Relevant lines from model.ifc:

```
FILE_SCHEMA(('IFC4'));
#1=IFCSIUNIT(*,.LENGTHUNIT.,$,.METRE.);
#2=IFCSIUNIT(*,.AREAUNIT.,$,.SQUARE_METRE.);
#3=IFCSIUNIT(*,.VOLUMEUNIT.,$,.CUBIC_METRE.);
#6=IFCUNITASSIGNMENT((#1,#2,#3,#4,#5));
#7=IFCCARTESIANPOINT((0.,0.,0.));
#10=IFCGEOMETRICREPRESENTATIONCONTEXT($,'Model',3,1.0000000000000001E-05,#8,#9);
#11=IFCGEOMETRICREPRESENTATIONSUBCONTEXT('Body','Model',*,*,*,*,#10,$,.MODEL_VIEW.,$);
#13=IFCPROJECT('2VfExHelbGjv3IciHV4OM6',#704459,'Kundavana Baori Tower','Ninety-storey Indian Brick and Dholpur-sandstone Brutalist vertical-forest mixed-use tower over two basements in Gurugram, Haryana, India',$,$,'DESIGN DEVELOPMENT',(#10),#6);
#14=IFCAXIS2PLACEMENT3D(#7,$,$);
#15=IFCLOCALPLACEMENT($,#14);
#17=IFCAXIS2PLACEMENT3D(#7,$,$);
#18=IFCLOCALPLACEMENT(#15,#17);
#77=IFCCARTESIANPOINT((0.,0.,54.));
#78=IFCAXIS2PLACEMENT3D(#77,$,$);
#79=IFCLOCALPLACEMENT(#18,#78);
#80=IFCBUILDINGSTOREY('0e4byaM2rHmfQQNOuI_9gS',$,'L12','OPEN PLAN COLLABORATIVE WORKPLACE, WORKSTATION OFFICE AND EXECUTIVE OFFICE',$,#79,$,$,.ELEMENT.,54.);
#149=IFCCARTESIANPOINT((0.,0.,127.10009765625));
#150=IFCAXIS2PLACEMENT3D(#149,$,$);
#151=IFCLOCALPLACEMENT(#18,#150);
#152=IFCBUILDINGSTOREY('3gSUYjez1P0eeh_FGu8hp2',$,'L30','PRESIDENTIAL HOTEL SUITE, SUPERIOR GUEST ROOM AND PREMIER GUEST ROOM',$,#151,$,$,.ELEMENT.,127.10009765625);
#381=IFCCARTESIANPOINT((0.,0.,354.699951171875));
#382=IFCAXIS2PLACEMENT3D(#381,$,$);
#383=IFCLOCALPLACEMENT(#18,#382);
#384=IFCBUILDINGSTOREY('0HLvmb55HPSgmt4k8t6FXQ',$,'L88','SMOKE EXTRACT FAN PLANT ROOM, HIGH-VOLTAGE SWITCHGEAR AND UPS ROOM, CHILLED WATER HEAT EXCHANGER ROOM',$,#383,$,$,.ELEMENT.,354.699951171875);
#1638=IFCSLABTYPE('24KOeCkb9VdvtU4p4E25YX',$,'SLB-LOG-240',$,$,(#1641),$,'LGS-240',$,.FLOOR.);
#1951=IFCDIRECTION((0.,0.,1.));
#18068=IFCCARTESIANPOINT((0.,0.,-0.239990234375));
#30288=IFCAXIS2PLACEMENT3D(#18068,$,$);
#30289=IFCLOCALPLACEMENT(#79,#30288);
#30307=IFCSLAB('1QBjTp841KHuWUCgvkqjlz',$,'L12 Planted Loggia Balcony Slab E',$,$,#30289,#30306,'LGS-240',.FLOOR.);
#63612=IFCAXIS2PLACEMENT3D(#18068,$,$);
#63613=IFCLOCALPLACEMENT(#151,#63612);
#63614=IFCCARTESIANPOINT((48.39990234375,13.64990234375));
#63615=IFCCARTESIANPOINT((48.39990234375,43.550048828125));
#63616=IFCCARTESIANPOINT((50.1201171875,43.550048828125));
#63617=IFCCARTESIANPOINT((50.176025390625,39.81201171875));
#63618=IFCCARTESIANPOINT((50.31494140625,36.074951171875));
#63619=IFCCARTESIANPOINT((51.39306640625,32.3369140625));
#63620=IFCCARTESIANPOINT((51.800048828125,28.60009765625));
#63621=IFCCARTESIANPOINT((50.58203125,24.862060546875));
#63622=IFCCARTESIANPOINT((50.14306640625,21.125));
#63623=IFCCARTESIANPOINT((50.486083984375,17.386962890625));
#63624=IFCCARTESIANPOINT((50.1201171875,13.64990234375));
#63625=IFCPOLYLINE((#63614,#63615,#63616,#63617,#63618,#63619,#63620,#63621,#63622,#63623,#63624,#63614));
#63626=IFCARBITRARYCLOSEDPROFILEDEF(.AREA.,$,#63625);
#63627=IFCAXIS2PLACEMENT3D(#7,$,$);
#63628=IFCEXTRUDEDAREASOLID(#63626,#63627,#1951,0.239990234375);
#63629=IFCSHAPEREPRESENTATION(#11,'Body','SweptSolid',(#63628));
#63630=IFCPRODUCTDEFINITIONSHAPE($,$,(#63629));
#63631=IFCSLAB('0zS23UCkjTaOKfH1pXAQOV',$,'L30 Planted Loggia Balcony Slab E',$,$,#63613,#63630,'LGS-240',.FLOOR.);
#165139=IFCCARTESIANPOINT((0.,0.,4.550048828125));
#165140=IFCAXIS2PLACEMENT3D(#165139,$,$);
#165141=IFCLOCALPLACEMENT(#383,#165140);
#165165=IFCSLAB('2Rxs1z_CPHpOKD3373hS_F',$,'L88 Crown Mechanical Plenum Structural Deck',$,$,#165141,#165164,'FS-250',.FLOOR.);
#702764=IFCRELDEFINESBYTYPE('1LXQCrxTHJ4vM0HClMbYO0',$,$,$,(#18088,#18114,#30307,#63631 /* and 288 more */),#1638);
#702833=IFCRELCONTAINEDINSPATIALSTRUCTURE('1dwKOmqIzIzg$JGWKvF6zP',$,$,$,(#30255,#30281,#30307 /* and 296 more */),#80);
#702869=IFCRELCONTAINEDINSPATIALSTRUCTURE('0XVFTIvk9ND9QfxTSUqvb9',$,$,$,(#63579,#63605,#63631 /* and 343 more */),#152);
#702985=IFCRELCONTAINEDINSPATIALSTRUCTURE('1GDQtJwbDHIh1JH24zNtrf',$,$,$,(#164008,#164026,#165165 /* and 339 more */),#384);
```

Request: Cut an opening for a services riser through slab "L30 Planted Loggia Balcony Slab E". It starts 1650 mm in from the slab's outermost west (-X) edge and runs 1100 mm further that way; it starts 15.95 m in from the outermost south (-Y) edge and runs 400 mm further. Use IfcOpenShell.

```python
import numpy as np
import ifcopenshell
import ifcopenshell.api.feature
import ifcopenshell.api.geometry
import ifcopenshell.api.root
import ifcopenshell.geom
import ifcopenshell.util.placement
import ifcopenshell.util.representation
import ifcopenshell.util.shape
import ifcopenshell.util.unit

model = ifcopenshell.open("model.ifc")
unit_scale = ifcopenshell.util.unit.calculate_unit_scale(model)
settings = ifcopenshell.geom.settings()


def volume(element):
    """Net volume in cubic metres, openings subtracted."""
    shape = ifcopenshell.geom.create_shape(settings, element)
    return ifcopenshell.util.shape.get_volume(shape.geometry)


slab = model.by_guid("0zS23UCkjTaOKfH1pXAQOV")
before = volume(slab)

# Extent in the slab's own axes, in metres. The edges named are its -X and -Y sides.
slab_shape = ifcopenshell.geom.create_shape(settings, slab)
vertices = ifcopenshell.util.shape.get_vertices(slab_shape.geometry)
x_min, y_min, bottom = vertices.min(axis=0)
top = vertices[:, 2].max()

opening = ifcopenshell.api.root.create_entity(model, ifc_class="IfcOpeningElement", name="Services riser opening", predefined_type="OPENING")
context = ifcopenshell.util.representation.get_context(model, "Model", "Body", "MODEL_VIEW")
width, depth = 1.1, 0.4
outline = [(0.0, 0.0), (width, 0.0), (width, depth), (0.0, depth), (0.0, 0.0)]
# Overshoot both faces by 50 mm so the cut is clean.
shape = ifcopenshell.api.geometry.add_slab_representation(
    model, context=context, depth=top - bottom + 0.1, polyline=outline
)
ifcopenshell.api.geometry.assign_representation(model, product=opening, representation=shape)

matrix = ifcopenshell.util.placement.get_local_placement(slab.ObjectPlacement)
matrix[:, 3] = matrix @ np.append(np.array([x_min + 1.65, y_min + 15.95, bottom - 0.05]) / unit_scale, 1.0)
ifcopenshell.api.geometry.edit_object_placement(model, product=opening, matrix=matrix, is_si=False)
ifcopenshell.api.feature.add_feature(model, feature=opening, element=slab)

after = volume(slab)

print(f"slab volume {before:.3f} -> {after:.3f} m3")

model.write("model_edited.ifc")
```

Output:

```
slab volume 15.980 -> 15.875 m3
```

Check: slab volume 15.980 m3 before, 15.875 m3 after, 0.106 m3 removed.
